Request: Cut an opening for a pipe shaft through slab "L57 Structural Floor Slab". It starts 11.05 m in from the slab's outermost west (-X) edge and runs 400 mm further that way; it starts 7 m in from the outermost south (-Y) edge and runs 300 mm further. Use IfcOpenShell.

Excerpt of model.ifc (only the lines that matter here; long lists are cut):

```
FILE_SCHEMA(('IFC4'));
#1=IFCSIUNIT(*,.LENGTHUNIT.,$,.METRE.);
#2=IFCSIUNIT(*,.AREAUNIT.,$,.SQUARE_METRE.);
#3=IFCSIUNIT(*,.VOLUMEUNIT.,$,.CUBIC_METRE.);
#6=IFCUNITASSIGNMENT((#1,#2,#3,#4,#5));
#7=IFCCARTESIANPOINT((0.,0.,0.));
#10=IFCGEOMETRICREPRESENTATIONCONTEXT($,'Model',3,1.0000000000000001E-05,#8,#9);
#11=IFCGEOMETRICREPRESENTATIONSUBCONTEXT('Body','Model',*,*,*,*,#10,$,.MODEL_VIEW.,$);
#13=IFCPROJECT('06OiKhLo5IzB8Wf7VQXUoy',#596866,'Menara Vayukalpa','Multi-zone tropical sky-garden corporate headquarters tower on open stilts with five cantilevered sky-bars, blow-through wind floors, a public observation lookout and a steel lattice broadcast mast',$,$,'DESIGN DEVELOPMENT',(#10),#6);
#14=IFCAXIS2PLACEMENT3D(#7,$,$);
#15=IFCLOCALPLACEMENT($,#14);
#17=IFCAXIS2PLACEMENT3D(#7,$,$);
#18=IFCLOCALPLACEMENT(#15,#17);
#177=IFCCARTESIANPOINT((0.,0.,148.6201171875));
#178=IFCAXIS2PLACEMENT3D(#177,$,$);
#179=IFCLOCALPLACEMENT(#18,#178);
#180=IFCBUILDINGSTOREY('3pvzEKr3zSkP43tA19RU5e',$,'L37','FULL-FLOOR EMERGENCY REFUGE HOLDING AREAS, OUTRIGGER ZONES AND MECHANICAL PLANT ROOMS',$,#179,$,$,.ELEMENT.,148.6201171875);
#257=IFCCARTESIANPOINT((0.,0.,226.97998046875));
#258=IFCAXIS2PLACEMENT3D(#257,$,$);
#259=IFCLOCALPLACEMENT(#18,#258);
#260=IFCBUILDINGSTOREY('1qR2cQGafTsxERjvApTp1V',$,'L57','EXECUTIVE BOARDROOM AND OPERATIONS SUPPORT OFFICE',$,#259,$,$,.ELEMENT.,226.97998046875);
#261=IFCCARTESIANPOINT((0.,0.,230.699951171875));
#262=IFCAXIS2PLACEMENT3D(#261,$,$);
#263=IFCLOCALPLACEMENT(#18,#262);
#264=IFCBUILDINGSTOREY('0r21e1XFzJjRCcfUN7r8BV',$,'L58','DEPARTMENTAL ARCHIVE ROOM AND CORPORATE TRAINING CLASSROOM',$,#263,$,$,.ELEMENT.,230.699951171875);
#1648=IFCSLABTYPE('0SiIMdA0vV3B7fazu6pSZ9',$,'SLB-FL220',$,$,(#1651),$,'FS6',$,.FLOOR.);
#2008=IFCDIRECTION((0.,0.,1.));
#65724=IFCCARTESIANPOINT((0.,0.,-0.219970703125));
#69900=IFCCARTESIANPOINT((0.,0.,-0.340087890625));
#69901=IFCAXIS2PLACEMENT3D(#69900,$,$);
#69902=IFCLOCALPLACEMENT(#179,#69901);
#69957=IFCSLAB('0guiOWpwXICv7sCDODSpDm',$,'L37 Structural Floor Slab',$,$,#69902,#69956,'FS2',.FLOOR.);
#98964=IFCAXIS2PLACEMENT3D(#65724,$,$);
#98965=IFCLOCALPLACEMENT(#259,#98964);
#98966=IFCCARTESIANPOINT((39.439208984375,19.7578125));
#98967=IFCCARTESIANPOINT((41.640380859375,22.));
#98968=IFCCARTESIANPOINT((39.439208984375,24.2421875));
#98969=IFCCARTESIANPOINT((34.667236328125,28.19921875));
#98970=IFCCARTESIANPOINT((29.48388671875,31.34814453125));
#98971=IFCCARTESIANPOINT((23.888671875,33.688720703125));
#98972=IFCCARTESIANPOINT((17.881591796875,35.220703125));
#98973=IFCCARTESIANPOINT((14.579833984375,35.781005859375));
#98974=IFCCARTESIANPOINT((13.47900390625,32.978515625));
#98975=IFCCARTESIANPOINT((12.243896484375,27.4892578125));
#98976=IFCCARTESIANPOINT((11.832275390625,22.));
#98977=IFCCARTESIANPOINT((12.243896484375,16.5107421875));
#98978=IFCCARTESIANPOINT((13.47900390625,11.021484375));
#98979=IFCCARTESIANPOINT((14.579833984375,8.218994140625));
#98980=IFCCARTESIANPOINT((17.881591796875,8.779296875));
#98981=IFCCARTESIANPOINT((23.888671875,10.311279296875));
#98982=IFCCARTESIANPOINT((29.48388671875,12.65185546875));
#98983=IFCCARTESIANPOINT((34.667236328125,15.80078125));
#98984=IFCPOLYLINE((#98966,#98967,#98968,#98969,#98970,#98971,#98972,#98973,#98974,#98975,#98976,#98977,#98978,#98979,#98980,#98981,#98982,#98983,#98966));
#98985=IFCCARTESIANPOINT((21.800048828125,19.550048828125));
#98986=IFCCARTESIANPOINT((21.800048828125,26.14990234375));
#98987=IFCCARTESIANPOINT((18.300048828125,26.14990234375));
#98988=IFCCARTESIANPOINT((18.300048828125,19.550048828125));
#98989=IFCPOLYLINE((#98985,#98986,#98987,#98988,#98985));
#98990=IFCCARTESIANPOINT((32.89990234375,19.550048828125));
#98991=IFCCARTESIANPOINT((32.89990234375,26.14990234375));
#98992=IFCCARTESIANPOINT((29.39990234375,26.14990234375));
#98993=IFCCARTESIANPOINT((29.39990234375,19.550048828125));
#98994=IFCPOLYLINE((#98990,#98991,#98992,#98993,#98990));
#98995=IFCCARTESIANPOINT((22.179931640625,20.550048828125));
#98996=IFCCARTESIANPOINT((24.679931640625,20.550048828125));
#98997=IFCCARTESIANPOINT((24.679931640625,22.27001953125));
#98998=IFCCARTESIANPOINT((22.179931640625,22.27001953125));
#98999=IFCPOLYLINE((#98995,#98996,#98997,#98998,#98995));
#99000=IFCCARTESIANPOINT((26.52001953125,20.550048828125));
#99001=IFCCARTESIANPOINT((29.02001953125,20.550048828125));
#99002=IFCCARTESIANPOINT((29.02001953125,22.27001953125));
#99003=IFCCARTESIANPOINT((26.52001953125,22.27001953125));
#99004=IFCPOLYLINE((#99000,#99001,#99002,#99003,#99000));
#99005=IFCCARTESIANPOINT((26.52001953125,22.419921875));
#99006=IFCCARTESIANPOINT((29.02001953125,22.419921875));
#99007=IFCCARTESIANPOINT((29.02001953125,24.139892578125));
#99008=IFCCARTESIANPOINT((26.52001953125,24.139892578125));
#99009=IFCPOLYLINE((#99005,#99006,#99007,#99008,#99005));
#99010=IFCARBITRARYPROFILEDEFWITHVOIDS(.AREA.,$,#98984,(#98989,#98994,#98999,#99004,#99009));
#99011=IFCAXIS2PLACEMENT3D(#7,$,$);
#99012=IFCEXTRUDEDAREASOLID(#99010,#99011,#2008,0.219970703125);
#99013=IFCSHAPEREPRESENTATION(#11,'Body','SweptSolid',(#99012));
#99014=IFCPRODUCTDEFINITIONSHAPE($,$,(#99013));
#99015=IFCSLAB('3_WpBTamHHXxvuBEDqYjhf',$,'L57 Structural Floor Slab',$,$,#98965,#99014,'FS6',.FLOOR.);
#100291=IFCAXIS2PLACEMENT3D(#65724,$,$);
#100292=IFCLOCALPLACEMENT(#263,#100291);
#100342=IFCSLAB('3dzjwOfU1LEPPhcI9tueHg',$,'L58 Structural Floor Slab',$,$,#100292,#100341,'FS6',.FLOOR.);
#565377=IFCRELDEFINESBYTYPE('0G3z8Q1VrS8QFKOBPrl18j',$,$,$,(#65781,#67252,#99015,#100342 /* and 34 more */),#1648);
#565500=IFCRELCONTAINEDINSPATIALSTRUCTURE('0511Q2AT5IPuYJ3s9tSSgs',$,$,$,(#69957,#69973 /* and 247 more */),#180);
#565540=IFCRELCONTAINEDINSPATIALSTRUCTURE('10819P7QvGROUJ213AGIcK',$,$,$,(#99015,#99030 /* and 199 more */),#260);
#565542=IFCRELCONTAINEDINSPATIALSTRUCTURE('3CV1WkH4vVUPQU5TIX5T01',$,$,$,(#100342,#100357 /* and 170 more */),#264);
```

```python
import numpy as np
import ifcopenshell
import ifcopenshell.api.feature
import ifcopenshell.api.geometry
import ifcopenshell.api.root
import ifcopenshell.geom
import ifcopenshell.util.placement
import ifcopenshell.util.representation
import ifcopenshell.util.shape
import ifcopenshell.util.unit

model = ifcopenshell.open("model.ifc")
unit_scale = ifcopenshell.util.unit.calculate_unit_scale(model)
settings = ifcopenshell.geom.settings()


def volume(element):
    """Net volume in cubic metres, openings subtracted."""
    shape = ifcopenshell.geom.create_shape(settings, element)
    return ifcopenshell.util.shape.get_volume(shape.geometry)


slab = model.by_guid("3_WpBTamHHXxvuBEDqYjhf")
before = volume(slab)

# Extent in the slab's own axes, in metres. The edges named are its -X and -Y sides.
slab_shape = ifcopenshell.geom.create_shape(settings, slab)
vertices = ifcopenshell.util.shape.get_vertices(slab_shape.geometry)
x_min, y_min, bottom = vertices.min(axis=0)
top = vertices[:, 2].max()

opening = ifcopenshell.api.root.create_entity(model, ifc_class="IfcOpeningElement", name="Pipe shaft opening", predefined_type="OPENING")
context = ifcopenshell.util.representation.get_context(model, "Model", "Body", "MODEL_VIEW")
width, depth = 0.4, 0.3
outline = [(0.0, 0.0), (width, 0.0), (width, depth), (0.0, depth), (0.0, 0.0)]
# Overshoot both faces by 50 mm so the cut is clean.
shape = ifcopenshell.api.geometry.add_slab_representation(
    model, context=context, depth=top - bottom + 0.1, polyline=outline
)
ifcopenshell.api.geometry.assign_representation(model, product=opening, representation=shape)

matrix = ifcopenshell.util.placement.get_local_placement(slab.ObjectPlacement)
matrix[:, 3] = matrix @ np.append(np.array([x_min + 11.05, y_min + 7, bottom - 0.05]) / unit_scale, 1.0)
ifcopenshell.api.geometry.edit_object_placement(model, product=opening, matrix=matrix, is_si=False)
ifcopenshell.api.feature.add_feature(model, feature=opening, element=slab)

after = volume(slab)

print(f"slab volume {before:.3f} -> {after:.3f} m3")

model.write("model_updated.ifc")
```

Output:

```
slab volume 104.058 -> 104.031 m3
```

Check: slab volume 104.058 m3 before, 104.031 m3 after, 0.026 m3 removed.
